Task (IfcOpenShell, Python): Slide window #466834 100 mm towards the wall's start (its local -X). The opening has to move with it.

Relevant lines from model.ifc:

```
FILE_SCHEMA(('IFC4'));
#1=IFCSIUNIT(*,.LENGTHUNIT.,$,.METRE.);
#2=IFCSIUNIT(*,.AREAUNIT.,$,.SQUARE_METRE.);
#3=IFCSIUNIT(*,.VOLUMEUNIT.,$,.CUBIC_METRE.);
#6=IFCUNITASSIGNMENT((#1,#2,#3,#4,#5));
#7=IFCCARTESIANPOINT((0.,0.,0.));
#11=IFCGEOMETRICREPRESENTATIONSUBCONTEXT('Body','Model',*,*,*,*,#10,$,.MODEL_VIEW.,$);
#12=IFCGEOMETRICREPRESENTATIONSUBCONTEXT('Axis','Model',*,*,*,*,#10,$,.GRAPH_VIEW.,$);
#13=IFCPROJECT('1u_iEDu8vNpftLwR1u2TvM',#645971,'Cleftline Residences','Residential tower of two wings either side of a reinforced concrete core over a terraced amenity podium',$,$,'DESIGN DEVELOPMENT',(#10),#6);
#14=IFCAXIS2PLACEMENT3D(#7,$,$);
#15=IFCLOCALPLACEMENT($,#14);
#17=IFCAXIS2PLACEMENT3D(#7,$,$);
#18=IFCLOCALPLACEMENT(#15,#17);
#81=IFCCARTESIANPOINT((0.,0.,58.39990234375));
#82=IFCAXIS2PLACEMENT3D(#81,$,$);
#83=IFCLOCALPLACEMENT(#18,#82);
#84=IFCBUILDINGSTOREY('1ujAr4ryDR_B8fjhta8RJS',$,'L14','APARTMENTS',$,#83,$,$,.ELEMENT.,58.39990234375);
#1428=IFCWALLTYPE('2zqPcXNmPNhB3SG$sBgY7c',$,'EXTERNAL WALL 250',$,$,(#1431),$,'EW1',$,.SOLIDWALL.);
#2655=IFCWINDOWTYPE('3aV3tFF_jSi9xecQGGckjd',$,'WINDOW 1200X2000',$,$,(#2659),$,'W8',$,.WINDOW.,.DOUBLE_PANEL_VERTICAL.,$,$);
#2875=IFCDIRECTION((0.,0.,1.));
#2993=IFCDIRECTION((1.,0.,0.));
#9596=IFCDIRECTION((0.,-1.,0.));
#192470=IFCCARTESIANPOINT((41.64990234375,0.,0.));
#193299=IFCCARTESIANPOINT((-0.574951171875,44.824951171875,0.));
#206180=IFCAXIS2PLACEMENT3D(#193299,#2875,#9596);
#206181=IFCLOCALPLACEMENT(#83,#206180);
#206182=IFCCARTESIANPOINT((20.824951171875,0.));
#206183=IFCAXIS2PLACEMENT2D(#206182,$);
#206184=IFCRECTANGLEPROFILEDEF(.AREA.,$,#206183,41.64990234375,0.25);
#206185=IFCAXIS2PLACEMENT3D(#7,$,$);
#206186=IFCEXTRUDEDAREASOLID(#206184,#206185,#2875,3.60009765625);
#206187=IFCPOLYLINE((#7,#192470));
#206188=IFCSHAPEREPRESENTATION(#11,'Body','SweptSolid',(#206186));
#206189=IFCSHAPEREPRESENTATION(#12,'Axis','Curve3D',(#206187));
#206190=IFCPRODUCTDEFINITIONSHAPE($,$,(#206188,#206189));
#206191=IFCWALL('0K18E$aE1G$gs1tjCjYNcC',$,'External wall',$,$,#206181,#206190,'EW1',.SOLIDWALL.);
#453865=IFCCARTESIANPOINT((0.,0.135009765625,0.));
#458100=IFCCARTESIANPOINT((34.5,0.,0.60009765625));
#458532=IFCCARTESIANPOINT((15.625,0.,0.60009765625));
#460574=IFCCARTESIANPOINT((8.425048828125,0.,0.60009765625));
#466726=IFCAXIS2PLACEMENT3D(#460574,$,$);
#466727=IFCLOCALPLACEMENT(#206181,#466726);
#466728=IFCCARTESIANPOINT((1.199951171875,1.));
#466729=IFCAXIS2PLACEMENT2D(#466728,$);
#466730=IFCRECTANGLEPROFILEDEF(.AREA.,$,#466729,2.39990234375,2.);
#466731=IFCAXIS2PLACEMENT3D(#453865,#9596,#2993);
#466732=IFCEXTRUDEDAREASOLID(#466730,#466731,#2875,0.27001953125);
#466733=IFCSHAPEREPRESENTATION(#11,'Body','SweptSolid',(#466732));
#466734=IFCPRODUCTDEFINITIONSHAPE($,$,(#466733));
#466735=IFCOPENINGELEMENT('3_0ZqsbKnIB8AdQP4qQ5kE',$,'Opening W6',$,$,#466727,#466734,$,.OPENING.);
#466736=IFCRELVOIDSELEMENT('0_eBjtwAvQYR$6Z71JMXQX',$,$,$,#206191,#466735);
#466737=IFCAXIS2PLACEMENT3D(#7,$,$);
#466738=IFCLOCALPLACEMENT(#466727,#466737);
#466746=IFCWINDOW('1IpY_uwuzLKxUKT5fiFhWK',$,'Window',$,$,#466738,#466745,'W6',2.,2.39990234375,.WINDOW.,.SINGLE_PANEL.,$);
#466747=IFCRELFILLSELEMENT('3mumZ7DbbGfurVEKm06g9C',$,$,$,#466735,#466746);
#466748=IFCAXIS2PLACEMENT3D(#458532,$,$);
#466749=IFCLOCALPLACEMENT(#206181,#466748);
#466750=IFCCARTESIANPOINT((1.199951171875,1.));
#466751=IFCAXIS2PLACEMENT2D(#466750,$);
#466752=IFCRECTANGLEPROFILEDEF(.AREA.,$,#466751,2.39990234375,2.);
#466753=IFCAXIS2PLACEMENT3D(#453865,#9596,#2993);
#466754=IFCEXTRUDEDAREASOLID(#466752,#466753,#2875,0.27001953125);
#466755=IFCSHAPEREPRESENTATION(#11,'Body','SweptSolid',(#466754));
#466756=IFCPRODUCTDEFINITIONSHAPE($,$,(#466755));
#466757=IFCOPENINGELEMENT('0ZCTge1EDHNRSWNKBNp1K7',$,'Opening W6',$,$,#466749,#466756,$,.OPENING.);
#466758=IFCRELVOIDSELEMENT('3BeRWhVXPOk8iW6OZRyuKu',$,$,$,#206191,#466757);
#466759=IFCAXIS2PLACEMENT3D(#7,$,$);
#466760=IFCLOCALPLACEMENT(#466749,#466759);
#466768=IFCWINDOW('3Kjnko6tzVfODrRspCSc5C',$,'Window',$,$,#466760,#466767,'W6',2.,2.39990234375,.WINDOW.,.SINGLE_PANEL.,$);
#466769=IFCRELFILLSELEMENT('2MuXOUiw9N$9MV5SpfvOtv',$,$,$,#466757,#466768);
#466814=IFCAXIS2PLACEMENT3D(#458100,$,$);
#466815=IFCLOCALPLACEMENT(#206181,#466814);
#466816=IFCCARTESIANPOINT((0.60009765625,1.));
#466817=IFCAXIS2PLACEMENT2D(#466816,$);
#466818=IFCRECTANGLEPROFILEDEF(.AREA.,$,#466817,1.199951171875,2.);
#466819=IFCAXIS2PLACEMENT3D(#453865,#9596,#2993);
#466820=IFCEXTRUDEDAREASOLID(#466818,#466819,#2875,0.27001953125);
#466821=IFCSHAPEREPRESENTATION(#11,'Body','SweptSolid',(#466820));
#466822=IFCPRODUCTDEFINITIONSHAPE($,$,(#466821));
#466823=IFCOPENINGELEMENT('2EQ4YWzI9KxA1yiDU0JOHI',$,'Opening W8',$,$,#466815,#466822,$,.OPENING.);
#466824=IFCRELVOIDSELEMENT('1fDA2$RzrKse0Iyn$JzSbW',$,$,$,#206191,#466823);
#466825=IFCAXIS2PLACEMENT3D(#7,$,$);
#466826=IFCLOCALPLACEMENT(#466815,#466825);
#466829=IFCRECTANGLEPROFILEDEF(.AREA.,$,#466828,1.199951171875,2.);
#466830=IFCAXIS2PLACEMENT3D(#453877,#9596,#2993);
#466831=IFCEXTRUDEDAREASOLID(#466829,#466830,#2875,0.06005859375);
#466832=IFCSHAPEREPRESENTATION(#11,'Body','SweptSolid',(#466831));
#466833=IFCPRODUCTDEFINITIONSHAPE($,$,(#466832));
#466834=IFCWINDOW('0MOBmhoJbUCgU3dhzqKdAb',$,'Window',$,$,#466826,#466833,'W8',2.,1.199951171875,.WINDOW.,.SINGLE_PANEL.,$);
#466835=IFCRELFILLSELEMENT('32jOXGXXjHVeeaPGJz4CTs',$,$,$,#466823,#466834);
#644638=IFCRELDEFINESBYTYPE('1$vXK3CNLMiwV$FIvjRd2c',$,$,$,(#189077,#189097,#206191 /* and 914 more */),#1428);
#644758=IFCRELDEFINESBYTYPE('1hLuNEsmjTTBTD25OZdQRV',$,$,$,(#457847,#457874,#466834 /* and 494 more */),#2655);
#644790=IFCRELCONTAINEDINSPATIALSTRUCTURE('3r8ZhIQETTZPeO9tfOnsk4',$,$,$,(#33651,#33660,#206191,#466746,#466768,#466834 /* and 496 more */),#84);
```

```python
import ifcopenshell
import ifcopenshell.api.geometry
import ifcopenshell.util.placement

model = ifcopenshell.open("model.ifc")

window = model.by_guid("0MOBmhoJbUCgU3dhzqKdAb")
opening = window.FillsVoids[0].RelatingOpeningElement
wall = opening.VoidsElements[0].RelatingBuildingElement

wall_matrix = ifcopenshell.util.placement.get_local_placement(wall.ObjectPlacement)
shift = wall_matrix[:3, 0] * -0.1
before = ifcopenshell.util.placement.get_local_placement(window.ObjectPlacement)[:3, 3].copy()

# The window is placed relative to its opening, so it follows when the opening moves.
matrix = ifcopenshell.util.placement.get_local_placement(opening.ObjectPlacement)
matrix[:3, 3] += shift
ifcopenshell.api.geometry.edit_object_placement(
    model, product=opening, matrix=matrix, is_si=False, should_transform_children=True
)

after = ifcopenshell.util.placement.get_local_placement(window.ObjectPlacement)[:3, 3]
print("window moved by", (after - before).round(3) + 0.0)

model.write("model_v2.ifc")
```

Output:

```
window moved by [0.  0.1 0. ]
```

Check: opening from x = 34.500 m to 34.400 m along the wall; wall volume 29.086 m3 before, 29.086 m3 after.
